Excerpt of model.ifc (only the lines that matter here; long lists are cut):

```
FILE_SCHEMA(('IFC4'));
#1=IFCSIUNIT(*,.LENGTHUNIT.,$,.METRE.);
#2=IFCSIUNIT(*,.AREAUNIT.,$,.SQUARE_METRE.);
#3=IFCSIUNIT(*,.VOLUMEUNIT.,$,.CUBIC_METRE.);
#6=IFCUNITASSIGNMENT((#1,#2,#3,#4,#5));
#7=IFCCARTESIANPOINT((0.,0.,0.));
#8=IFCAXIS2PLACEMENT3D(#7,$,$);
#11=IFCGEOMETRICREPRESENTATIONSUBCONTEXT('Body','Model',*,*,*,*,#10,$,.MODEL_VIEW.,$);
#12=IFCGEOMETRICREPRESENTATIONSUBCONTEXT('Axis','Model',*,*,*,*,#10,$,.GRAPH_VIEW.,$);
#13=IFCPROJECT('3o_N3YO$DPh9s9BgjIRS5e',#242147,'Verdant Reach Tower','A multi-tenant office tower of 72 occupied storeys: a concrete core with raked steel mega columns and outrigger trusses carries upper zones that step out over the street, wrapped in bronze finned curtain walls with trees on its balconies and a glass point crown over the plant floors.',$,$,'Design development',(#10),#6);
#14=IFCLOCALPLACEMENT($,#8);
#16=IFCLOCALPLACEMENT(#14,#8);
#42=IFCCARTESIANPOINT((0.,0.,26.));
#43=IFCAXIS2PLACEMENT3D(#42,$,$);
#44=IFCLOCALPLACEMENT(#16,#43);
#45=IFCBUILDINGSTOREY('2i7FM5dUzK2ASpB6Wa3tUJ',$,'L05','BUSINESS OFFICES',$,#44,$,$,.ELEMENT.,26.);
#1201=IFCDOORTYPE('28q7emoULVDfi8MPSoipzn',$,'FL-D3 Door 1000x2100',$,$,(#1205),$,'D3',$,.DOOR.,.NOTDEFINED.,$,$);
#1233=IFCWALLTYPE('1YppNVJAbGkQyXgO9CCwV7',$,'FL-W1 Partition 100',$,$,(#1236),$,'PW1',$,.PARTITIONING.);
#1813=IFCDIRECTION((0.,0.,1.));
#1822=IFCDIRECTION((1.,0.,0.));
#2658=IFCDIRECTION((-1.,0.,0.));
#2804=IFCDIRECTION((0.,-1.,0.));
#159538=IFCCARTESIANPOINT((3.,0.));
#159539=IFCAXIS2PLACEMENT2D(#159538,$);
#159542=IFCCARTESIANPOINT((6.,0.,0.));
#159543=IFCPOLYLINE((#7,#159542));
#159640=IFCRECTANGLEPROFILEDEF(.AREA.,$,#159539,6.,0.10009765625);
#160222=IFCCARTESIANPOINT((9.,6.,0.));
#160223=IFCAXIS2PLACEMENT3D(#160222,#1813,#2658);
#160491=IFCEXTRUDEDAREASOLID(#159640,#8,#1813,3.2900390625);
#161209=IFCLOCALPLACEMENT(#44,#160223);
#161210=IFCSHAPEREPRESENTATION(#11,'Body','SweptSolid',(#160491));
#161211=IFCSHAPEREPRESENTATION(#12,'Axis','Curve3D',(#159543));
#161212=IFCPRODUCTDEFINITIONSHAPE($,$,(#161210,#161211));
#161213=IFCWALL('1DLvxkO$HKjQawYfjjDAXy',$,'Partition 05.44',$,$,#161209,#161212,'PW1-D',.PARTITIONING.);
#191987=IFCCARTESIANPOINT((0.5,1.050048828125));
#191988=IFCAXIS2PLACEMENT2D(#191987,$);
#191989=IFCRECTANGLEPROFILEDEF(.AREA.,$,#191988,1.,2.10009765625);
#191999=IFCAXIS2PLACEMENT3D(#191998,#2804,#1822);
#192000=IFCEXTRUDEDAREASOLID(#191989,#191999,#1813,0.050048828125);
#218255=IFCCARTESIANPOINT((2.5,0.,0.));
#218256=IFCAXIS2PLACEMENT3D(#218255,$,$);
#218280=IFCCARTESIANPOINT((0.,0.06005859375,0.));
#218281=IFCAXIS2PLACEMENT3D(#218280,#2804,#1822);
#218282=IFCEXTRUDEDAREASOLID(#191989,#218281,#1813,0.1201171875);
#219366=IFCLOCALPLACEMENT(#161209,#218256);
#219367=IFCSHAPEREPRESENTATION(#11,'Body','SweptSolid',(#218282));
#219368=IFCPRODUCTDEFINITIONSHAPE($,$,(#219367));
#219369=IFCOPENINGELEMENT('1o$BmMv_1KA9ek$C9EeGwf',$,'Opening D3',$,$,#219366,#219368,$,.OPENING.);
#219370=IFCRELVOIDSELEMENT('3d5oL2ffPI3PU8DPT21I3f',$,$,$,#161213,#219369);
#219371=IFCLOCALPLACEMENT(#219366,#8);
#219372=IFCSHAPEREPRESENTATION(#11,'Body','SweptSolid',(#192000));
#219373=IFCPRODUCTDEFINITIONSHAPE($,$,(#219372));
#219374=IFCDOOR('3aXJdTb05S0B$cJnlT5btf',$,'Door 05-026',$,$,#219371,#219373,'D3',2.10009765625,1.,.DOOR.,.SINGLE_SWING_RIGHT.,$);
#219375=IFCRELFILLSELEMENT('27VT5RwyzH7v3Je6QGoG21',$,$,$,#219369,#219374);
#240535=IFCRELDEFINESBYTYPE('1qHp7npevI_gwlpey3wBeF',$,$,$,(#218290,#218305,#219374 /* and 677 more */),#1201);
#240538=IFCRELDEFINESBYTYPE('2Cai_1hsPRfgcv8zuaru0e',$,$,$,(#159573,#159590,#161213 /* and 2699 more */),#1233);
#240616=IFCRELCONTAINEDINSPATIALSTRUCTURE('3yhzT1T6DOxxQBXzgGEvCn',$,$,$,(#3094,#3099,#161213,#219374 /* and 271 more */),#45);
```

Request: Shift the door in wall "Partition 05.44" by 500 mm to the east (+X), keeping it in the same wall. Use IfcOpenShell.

```python
import ifcopenshell
import ifcopenshell.api.geometry
import ifcopenshell.util.placement

model = ifcopenshell.open("model.ifc")

door = model.by_guid("3aXJdTb05S0B$cJnlT5btf")
opening = door.FillsVoids[0].RelatingOpeningElement
wall = opening.VoidsElements[0].RelatingBuildingElement

wall_matrix = ifcopenshell.util.placement.get_local_placement(wall.ObjectPlacement)
shift = wall_matrix[:3, 0] * -0.5
before = ifcopenshell.util.placement.get_local_placement(door.ObjectPlacement)[:3, 3].copy()

# The door is placed relative to its opening, so it follows when the opening moves.
matrix = ifcopenshell.util.placement.get_local_placement(opening.ObjectPlacement)
matrix[:3, 3] += shift
ifcopenshell.api.geometry.edit_object_placement(
    model, product=opening, matrix=matrix, is_si=False, should_transform_children=True
)

after = ifcopenshell.util.placement.get_local_placement(door.ObjectPlacement)[:3, 3]
print("door moved by", (after - before).round(3) + 0.0)

model.write("model-out.ifc")
```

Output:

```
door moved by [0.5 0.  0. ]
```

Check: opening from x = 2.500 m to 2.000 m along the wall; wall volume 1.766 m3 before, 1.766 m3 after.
